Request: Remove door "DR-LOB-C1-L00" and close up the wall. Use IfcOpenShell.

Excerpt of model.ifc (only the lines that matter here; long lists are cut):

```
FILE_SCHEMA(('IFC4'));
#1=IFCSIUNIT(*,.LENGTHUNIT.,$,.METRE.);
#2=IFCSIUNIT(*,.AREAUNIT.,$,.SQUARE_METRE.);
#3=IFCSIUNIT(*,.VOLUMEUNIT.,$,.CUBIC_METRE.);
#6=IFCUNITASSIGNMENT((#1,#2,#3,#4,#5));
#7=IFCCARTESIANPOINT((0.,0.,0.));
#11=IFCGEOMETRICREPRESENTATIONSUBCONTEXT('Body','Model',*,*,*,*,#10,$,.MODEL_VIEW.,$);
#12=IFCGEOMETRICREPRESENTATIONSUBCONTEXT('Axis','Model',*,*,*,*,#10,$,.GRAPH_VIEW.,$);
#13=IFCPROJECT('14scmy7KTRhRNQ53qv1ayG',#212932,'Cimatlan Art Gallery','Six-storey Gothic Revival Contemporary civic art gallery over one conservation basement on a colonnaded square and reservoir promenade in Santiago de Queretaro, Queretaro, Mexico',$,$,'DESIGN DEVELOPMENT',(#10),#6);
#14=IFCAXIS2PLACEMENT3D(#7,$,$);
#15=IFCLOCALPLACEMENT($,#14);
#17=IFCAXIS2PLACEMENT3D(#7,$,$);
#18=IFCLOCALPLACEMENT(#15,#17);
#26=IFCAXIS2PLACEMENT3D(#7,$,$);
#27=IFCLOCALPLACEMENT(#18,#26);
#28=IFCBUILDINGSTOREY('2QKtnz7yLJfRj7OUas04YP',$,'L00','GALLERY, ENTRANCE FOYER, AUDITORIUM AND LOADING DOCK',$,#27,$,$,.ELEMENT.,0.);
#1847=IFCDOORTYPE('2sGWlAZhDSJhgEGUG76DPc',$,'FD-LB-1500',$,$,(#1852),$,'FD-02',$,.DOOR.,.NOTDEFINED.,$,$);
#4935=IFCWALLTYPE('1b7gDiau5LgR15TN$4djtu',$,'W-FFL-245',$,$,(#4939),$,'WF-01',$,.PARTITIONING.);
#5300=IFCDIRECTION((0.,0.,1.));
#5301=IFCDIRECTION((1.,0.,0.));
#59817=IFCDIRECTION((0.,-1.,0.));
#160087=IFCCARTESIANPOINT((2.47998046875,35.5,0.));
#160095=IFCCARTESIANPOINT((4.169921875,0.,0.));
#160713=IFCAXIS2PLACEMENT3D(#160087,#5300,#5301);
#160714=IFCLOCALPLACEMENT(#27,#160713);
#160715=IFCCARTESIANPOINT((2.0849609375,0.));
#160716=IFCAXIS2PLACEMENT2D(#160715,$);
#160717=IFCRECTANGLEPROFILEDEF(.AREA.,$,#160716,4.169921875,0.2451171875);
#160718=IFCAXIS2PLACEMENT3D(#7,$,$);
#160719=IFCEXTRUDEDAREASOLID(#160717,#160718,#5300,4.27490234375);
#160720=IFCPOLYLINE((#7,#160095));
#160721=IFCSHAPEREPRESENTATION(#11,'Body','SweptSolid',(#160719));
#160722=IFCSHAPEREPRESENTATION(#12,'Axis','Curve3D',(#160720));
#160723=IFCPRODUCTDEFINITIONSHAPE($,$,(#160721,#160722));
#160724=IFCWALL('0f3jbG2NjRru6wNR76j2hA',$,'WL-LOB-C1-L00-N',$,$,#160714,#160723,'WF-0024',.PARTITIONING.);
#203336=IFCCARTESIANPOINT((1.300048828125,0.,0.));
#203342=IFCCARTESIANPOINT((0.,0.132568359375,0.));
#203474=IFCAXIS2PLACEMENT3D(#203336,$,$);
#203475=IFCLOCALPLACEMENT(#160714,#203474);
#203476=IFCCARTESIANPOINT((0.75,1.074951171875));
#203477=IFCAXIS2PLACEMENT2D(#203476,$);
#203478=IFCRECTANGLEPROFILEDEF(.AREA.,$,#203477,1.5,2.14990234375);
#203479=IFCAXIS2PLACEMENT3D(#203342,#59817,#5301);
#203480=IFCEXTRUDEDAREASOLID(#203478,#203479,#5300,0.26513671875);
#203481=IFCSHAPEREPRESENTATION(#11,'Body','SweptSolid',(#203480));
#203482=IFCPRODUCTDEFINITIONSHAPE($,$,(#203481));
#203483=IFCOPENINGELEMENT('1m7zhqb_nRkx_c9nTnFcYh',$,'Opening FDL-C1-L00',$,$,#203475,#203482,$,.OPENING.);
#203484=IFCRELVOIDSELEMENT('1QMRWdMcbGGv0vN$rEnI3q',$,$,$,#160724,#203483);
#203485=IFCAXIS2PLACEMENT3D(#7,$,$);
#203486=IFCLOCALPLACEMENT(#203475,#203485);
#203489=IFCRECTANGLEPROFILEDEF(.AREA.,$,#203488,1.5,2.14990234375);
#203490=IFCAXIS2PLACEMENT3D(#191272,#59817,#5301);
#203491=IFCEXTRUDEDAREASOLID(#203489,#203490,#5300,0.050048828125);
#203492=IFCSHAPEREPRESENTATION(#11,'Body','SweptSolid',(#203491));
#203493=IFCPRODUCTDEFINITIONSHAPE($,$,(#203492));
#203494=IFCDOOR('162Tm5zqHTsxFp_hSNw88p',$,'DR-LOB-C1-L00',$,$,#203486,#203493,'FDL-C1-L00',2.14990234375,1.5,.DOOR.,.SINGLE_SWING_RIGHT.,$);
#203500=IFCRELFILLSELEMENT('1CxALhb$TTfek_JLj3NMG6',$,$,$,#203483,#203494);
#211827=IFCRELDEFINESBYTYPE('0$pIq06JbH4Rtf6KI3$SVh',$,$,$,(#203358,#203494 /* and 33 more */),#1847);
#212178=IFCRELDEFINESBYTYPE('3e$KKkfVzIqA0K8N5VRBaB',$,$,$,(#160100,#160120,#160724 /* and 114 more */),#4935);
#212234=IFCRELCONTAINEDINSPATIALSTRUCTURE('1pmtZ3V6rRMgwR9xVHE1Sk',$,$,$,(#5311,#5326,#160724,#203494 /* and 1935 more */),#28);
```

```python
import ifcopenshell
import ifcopenshell.api.feature
import ifcopenshell.api.root
import ifcopenshell.geom
import ifcopenshell.util.shape

model = ifcopenshell.open("model.ifc")
settings = ifcopenshell.geom.settings()


def volume(element):
    """Net volume in cubic metres, openings subtracted."""
    shape = ifcopenshell.geom.create_shape(settings, element)
    return ifcopenshell.util.shape.get_volume(shape.geometry)


door = model.by_id(203494)
opening = door.FillsVoids[0].RelatingOpeningElement
wall = opening.VoidsElements[0].RelatingBuildingElement
before = volume(wall)

ifcopenshell.api.root.remove_product(model, product=door)
ifcopenshell.api.feature.remove_feature(model, feature=opening)

after = volume(wall)

print(f"wall volume {before:.3f} -> {after:.3f} m3")

model.write("model_rev.ifc")
```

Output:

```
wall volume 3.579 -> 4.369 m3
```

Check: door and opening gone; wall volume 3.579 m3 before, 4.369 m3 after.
